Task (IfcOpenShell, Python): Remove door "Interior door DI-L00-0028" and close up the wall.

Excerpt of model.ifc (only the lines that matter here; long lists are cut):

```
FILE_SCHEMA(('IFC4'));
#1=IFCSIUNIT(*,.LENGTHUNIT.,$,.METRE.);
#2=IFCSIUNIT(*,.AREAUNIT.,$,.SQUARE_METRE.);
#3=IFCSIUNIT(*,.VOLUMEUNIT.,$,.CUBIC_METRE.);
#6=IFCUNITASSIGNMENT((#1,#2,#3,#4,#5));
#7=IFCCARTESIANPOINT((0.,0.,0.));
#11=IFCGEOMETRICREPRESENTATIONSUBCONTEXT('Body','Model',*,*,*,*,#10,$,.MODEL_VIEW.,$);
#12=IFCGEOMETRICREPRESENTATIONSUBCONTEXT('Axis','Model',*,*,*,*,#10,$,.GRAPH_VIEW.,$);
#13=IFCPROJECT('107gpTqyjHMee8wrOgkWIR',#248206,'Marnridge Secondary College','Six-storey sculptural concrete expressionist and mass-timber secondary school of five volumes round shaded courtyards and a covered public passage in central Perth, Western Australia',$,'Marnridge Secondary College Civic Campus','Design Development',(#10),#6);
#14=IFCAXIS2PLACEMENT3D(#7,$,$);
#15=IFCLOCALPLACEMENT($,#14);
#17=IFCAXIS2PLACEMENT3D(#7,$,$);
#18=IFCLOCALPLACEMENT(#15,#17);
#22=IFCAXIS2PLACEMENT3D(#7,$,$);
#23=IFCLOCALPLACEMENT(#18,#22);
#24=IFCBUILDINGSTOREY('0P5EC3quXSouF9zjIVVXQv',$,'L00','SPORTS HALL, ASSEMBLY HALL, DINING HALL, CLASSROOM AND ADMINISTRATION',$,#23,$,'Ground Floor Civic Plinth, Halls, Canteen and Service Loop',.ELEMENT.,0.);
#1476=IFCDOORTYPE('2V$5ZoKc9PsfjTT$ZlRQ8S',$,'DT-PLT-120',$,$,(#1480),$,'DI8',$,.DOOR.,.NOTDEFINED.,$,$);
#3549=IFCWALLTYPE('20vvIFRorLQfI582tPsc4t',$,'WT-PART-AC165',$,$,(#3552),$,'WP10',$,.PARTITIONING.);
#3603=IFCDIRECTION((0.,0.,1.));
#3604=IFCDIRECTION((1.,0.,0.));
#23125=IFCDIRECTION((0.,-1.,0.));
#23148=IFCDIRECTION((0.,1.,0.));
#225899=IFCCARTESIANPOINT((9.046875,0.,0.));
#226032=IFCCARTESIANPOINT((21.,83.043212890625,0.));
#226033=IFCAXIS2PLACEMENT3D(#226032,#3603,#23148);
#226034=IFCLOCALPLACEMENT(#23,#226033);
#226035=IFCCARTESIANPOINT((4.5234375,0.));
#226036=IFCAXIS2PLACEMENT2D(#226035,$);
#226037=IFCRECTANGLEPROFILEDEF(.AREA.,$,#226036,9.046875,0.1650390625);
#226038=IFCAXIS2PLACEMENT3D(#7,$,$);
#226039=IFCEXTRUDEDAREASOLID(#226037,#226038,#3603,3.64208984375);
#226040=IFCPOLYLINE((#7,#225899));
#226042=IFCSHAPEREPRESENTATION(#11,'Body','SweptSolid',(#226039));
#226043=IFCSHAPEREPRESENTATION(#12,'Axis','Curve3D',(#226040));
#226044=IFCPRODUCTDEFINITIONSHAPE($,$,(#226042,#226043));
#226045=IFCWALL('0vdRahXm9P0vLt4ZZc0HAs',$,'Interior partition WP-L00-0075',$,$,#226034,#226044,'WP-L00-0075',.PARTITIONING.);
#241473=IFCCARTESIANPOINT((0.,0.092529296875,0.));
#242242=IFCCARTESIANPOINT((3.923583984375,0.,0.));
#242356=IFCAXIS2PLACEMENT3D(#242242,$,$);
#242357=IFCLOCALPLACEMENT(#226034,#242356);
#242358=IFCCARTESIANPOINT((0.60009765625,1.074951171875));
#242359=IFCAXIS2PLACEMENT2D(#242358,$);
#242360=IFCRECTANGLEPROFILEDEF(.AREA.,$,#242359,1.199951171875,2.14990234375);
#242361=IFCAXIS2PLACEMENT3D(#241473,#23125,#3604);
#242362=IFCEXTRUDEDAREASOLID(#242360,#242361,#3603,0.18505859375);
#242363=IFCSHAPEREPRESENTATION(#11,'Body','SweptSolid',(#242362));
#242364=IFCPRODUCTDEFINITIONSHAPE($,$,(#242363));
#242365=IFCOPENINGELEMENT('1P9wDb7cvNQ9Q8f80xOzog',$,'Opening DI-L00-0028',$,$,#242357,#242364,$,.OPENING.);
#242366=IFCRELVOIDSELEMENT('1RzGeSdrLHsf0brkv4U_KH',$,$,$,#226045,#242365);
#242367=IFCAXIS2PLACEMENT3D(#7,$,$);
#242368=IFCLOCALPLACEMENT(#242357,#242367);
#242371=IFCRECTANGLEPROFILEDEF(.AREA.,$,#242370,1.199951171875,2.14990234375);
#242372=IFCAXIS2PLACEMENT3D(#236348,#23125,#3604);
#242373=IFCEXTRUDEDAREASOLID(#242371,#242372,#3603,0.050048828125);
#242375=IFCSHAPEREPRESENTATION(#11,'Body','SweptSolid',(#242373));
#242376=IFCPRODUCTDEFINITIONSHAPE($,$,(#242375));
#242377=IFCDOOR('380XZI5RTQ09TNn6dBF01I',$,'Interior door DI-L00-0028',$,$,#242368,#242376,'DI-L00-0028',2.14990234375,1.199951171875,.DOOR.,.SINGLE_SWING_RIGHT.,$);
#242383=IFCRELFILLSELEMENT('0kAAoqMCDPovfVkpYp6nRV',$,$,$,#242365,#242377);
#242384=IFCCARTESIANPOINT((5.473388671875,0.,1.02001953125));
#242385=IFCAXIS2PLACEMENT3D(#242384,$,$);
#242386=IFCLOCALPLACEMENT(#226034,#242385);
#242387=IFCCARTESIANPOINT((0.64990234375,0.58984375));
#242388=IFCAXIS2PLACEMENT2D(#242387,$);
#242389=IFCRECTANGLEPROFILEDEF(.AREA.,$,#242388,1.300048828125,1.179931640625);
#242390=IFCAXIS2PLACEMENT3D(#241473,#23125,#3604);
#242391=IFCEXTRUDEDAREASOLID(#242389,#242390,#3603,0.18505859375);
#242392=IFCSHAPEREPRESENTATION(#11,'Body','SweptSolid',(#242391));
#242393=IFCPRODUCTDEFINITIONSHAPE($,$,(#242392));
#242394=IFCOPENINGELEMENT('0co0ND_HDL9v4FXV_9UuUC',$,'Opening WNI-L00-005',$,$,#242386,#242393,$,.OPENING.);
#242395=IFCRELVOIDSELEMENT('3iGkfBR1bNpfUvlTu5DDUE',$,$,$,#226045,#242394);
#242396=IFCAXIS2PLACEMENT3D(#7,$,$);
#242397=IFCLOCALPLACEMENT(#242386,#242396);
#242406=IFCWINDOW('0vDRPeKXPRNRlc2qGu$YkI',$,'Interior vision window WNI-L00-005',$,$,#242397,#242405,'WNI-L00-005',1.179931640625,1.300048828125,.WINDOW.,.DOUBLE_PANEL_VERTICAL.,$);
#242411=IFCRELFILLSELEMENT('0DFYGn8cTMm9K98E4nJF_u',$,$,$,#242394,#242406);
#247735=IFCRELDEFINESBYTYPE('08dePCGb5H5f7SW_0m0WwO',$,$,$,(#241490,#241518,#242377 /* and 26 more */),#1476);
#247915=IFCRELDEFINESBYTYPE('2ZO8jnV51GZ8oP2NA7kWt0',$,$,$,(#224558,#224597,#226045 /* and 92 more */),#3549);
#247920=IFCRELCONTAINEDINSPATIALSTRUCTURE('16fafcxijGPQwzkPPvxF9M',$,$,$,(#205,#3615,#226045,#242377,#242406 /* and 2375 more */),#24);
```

```python
import ifcopenshell
import ifcopenshell.api.feature
import ifcopenshell.api.root
import ifcopenshell.geom
import ifcopenshell.util.shape

model = ifcopenshell.open("model.ifc")
settings = ifcopenshell.geom.settings()


def volume(element):
    """Net volume in cubic metres, openings subtracted."""
    shape = ifcopenshell.geom.create_shape(settings, element)
    return ifcopenshell.util.shape.get_volume(shape.geometry)


door = model.by_guid("380XZI5RTQ09TNn6dBF01I")
opening = door.FillsVoids[0].RelatingOpeningElement
wall = opening.VoidsElements[0].RelatingBuildingElement
before = volume(wall)

ifcopenshell.api.root.remove_product(model, product=door)
ifcopenshell.api.feature.remove_feature(model, feature=opening)

after = volume(wall)

print(f"wall volume {before:.3f} -> {after:.3f} m3")

model.write("model_edited.ifc")
```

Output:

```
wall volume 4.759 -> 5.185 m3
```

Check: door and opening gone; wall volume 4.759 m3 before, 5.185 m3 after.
